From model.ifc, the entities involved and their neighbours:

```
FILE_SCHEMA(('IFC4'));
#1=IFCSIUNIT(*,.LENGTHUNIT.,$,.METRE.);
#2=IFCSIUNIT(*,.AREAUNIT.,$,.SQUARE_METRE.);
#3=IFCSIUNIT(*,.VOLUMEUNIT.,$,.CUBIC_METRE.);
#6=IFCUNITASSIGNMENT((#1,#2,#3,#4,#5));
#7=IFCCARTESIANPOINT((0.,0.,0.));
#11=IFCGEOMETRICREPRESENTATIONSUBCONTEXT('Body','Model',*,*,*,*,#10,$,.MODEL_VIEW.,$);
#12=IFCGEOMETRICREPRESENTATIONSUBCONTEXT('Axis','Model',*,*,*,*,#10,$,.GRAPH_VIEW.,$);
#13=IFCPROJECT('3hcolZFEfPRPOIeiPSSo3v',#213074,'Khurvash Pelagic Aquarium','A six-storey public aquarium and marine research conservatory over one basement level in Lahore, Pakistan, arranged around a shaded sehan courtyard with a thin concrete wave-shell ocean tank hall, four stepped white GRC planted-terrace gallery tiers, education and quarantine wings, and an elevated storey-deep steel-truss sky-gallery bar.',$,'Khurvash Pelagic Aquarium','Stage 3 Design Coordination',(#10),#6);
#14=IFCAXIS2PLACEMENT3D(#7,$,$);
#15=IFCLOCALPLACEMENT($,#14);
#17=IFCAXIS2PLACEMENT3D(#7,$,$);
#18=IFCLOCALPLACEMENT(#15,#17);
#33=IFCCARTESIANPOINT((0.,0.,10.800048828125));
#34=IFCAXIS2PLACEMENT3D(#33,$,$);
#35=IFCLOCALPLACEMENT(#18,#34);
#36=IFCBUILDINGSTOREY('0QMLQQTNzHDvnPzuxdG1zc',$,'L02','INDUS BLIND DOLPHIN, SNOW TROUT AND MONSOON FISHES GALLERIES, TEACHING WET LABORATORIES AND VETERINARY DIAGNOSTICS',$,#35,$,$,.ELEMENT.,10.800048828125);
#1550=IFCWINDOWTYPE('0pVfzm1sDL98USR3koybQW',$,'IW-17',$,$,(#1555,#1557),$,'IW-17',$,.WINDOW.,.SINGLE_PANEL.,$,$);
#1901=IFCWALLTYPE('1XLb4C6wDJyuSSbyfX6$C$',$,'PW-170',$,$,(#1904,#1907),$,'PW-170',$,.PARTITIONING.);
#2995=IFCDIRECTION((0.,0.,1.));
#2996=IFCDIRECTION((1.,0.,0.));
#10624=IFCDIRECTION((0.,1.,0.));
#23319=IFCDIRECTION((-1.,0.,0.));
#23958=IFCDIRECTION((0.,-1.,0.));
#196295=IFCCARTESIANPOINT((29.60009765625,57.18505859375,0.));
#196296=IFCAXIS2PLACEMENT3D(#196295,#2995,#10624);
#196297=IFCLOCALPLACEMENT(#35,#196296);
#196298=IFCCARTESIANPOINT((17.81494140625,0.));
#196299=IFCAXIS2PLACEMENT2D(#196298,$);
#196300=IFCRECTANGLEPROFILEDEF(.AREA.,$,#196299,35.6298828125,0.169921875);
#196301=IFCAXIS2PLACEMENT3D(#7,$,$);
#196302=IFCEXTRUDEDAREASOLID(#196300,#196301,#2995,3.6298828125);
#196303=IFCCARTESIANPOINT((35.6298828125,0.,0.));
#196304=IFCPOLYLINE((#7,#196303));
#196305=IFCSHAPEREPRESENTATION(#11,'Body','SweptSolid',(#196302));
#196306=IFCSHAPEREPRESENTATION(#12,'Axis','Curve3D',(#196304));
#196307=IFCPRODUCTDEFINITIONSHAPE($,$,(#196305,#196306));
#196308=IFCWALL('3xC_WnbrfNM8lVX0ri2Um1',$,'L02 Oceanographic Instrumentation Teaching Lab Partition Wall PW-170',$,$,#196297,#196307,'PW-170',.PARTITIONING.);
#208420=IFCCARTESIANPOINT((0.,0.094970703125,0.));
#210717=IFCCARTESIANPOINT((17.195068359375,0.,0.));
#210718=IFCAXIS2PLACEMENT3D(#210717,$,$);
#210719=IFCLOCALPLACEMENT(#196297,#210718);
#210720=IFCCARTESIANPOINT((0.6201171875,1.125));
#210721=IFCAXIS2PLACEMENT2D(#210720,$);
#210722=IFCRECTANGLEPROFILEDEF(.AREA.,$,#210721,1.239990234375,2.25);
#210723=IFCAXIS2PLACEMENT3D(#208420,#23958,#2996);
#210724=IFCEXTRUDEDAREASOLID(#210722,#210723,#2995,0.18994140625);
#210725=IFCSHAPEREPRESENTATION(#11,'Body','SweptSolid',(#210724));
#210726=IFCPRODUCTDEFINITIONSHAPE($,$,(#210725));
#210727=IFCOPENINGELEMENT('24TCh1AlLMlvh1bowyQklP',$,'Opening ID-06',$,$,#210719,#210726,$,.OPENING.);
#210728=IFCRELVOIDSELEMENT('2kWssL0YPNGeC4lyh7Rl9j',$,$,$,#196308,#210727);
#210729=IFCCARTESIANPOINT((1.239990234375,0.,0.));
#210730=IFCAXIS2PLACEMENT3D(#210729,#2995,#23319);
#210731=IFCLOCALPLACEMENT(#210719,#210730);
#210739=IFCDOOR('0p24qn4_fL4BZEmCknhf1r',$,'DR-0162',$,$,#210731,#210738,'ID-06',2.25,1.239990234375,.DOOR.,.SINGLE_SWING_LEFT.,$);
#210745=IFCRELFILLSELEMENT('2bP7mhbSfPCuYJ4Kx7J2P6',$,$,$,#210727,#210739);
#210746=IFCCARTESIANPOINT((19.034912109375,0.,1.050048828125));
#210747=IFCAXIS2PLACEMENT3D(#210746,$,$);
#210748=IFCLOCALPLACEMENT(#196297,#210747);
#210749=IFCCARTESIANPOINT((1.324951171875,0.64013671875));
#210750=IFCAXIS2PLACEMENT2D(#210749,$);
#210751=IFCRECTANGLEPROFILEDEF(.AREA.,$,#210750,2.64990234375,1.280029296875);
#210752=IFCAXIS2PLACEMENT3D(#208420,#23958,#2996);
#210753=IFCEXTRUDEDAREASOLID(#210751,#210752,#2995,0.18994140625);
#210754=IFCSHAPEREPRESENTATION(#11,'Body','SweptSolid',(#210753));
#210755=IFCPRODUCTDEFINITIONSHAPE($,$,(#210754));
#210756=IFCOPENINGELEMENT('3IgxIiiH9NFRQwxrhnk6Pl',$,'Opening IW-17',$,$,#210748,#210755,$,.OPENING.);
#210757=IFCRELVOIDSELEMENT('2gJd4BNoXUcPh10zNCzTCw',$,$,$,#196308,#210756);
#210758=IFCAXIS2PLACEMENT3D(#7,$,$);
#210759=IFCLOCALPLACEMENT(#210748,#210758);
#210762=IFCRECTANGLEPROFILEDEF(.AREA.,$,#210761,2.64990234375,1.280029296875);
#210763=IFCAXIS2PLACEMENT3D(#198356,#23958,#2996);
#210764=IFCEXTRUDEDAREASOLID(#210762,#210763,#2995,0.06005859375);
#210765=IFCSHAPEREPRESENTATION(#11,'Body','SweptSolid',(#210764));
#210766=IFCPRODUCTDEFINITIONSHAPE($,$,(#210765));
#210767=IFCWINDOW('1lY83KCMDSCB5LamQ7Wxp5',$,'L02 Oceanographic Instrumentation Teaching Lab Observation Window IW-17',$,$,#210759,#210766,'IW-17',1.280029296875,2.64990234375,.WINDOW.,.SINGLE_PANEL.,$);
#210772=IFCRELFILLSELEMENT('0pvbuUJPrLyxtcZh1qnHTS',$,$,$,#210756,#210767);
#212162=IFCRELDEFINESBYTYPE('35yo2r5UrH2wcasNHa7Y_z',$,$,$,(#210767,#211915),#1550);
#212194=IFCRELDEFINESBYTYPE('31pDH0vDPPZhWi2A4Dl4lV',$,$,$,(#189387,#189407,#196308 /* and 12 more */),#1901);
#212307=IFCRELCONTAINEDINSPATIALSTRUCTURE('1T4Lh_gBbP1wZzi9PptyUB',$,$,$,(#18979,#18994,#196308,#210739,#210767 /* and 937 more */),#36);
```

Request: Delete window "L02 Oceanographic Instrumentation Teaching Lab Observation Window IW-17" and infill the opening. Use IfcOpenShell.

```python
import ifcopenshell
import ifcopenshell.api.feature
import ifcopenshell.api.root
import ifcopenshell.geom
import ifcopenshell.util.shape

model = ifcopenshell.open("model.ifc")
settings = ifcopenshell.geom.settings()


def volume(element):
    """Net volume in cubic metres, openings subtracted."""
    shape = ifcopenshell.geom.create_shape(settings, element)
    return ifcopenshell.util.shape.get_volume(shape.geometry)


window = model.by_guid("1lY83KCMDSCB5LamQ7Wxp5")
opening = window.FillsVoids[0].RelatingOpeningElement
wall = opening.VoidsElements[0].RelatingBuildingElement
before = volume(wall)

ifcopenshell.api.root.remove_product(model, product=window)
ifcopenshell.api.feature.remove_feature(model, feature=opening)

after = volume(wall)

print(f"wall volume {before:.3f} -> {after:.3f} m3")

model.write("model_updated.ifc")
```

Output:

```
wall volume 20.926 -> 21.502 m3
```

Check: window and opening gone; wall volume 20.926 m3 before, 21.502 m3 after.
